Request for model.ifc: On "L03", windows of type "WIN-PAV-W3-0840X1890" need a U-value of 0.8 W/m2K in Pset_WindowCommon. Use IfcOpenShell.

First a look at what the model holds.

```python
import ifcopenshell
import ifcopenshell.util.element

model = ifcopenshell.open("model.ifc")
print(model.schema)
storey = next(s for s in model.by_type("IfcBuildingStorey") if s.Name == "L03")
windows = [e for e in ifcopenshell.util.element.get_decomposition(storey) if e.is_a("IfcWindow")]
seen = {}
for e in windows:
    element_type = ifcopenshell.util.element.get_type(e)
    key = (element_type.Name if element_type != e and element_type else None, ifcopenshell.util.element.get_pset(e, "Pset_WindowCommon", "ThermalTransmittance"))
    seen[key] = seen.get(key, 0) + 1
for (name, value), count in sorted(seen.items(), key=str):
    print(count, "x", name, "|", value)
```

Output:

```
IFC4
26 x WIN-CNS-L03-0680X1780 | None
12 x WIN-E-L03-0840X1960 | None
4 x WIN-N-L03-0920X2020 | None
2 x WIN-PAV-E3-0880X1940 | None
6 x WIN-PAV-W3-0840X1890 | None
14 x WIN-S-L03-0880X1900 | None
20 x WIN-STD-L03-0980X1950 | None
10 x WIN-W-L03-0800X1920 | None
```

```python
import ifcopenshell
import ifcopenshell.api.pset
import ifcopenshell.util.element

model = ifcopenshell.open("model.ifc")

storey = next(s for s in model.by_type("IfcBuildingStorey") if s.Name == "L03")
windows = [e for e in ifcopenshell.util.element.get_decomposition(storey) if e.is_a("IfcWindow")]

count = 0
for e in windows:
    element_type = ifcopenshell.util.element.get_type(e)
    if element_type in (None, e) or element_type.Name != "WIN-PAV-W3-0840X1890":
        continue
    # add_pset returns the element's existing set when there is one.
    pset = ifcopenshell.api.pset.add_pset(model, product=e, name="Pset_WindowCommon")
    ifcopenshell.api.pset.edit_pset(model, pset=pset, properties={"ThermalTransmittance": 0.8})
    count += 1

print(count, "windows updated")

model.write("model_rev.ifc")
```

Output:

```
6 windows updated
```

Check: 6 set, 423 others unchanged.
